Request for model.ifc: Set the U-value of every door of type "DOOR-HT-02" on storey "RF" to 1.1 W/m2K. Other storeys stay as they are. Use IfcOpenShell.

First a look at what the model holds.

```python
import ifcopenshell
import ifcopenshell.util.element

model = ifcopenshell.open("model.ifc")
print(model.schema)
storey = next(s for s in model.by_type("IfcBuildingStorey") if s.Name == "RF")
doors = [e for e in ifcopenshell.util.element.get_decomposition(storey) if e.is_a("IfcDoor")]
seen = {}
for e in doors:
    element_type = ifcopenshell.util.element.get_type(e)
    key = (element_type.Name if element_type != e and element_type else None, ifcopenshell.util.element.get_pset(e, "Pset_DoorCommon", "ThermalTransmittance"))
    seen[key] = seen.get(key, 0) + 1
for (name, value), count in sorted(seen.items(), key=str):
    print(count, "x", name, "|", value)
```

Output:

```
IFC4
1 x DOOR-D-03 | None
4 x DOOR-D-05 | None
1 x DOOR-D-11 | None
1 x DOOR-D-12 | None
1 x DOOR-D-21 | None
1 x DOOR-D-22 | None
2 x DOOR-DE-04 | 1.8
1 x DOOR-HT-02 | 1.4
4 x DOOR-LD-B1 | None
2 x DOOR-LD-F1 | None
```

```python
import ifcopenshell
import ifcopenshell.api.pset
import ifcopenshell.util.element

model = ifcopenshell.open("model.ifc")

storey = next(s for s in model.by_type("IfcBuildingStorey") if s.Name == "RF")
doors = [e for e in ifcopenshell.util.element.get_decomposition(storey) if e.is_a("IfcDoor")]

count = 0
for e in doors:
    element_type = ifcopenshell.util.element.get_type(e)
    if element_type in (None, e) or element_type.Name != "DOOR-HT-02":
        continue
    # add_pset returns the element's existing set when there is one.
    pset = ifcopenshell.api.pset.add_pset(model, product=e, name="Pset_DoorCommon")
    ifcopenshell.api.pset.edit_pset(model, pset=pset, properties={"ThermalTransmittance": 1.1})
    count += 1

print(count, "doors updated")

model.write("model_rev.ifc")
```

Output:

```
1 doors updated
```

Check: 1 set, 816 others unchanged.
